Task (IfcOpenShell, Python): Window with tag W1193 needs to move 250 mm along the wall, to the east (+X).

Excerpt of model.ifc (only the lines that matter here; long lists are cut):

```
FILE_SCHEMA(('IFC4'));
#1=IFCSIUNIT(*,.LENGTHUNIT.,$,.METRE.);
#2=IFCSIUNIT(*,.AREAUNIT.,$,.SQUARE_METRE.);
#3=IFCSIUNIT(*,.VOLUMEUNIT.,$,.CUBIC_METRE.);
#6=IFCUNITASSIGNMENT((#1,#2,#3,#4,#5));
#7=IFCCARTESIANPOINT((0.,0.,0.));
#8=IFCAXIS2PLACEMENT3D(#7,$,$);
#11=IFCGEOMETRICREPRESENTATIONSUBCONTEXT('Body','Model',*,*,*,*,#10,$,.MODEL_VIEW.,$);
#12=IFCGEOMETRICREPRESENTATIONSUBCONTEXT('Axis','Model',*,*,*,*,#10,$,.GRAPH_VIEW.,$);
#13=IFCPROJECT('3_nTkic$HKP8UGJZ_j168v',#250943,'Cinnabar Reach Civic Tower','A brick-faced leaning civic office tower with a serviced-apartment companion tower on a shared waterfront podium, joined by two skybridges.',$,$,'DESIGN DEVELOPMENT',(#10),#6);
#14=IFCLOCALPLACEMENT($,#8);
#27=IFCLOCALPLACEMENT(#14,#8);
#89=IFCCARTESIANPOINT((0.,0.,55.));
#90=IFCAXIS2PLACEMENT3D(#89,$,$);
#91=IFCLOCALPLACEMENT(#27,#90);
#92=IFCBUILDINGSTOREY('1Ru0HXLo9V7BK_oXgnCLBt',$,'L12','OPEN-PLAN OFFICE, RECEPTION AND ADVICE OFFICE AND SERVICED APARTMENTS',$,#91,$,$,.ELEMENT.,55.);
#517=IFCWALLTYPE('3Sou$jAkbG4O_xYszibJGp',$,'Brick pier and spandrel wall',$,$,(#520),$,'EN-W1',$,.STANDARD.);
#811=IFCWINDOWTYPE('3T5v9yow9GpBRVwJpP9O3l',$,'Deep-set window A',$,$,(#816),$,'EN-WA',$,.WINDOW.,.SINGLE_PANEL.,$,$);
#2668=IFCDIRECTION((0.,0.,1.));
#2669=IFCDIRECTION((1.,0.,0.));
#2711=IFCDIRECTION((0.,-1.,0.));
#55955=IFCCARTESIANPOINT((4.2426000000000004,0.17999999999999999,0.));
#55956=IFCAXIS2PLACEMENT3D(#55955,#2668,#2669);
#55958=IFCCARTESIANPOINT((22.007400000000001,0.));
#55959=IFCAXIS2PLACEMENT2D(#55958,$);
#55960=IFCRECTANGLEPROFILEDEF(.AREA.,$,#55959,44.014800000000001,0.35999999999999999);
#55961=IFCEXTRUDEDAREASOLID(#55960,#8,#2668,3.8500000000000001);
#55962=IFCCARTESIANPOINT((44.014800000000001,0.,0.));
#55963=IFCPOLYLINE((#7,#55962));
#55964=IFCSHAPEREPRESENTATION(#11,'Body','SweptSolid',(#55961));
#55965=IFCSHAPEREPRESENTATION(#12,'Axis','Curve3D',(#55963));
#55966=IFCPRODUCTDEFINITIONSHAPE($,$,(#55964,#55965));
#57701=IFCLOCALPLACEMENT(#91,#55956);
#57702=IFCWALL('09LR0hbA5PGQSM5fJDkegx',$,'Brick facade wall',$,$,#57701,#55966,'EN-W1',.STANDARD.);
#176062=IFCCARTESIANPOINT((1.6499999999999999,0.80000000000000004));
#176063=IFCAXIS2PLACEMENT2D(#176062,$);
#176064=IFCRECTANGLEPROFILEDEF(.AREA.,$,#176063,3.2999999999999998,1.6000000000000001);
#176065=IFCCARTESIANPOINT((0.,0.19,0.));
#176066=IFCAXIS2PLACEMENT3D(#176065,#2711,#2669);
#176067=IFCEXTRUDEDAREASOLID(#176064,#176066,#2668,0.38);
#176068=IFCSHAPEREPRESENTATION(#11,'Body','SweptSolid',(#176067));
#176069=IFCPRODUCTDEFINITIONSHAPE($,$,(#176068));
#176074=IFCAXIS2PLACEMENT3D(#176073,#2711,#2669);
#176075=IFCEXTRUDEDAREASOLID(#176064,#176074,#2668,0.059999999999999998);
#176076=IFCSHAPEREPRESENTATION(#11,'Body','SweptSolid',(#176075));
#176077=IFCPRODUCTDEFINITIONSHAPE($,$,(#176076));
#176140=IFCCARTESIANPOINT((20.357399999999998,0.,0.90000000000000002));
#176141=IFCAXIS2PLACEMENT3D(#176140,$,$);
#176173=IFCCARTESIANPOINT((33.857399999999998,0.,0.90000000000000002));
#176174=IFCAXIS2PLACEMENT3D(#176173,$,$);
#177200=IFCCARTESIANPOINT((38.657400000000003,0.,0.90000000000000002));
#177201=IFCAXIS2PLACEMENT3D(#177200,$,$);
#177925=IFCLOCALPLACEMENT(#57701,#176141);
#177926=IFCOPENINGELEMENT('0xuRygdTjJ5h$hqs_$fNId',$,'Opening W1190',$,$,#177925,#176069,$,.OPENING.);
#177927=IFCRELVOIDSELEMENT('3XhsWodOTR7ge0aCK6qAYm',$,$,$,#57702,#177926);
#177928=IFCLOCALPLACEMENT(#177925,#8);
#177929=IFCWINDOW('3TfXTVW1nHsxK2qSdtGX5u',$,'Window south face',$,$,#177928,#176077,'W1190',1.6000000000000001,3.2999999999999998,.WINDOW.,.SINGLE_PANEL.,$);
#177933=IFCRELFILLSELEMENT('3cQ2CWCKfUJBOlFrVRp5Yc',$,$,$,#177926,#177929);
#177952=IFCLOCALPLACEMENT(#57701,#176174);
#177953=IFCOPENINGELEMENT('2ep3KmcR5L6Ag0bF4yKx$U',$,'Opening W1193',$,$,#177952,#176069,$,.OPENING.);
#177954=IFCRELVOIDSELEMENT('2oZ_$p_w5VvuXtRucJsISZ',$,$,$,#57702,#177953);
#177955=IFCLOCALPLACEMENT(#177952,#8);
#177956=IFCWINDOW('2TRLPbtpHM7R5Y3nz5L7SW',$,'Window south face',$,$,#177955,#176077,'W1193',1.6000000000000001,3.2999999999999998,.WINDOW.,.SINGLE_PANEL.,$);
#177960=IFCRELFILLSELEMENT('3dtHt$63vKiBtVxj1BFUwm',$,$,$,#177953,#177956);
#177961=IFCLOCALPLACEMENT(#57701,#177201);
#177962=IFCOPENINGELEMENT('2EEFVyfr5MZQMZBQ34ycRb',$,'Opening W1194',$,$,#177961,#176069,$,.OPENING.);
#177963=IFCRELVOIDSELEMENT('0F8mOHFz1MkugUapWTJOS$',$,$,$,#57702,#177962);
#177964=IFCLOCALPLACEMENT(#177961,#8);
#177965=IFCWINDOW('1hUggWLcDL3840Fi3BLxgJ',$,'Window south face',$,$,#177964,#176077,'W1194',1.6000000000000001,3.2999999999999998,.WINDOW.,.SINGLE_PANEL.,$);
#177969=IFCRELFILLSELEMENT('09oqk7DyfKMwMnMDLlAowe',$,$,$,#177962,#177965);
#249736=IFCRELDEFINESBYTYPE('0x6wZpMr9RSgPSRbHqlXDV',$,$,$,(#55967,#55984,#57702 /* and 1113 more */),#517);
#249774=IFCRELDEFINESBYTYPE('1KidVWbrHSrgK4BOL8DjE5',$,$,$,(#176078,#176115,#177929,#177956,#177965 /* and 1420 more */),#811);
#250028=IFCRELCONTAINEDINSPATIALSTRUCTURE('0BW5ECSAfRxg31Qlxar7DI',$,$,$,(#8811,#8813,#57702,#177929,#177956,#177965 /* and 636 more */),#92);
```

```python
import ifcopenshell
import ifcopenshell.api.geometry
import ifcopenshell.util.placement
import ifcopenshell.util.unit

model = ifcopenshell.open("model.ifc")
unit_scale = ifcopenshell.util.unit.calculate_unit_scale(model)

window = model.by_guid("2TRLPbtpHM7R5Y3nz5L7SW")
opening = window.FillsVoids[0].RelatingOpeningElement
wall = opening.VoidsElements[0].RelatingBuildingElement

wall_matrix = ifcopenshell.util.placement.get_local_placement(wall.ObjectPlacement)
shift = wall_matrix[:3, 0] * 0.25 / unit_scale
before = ifcopenshell.util.placement.get_local_placement(window.ObjectPlacement)[:3, 3].copy()

# The window is placed relative to its opening, so it follows when the opening moves.
matrix = ifcopenshell.util.placement.get_local_placement(opening.ObjectPlacement)
matrix[:3, 3] += shift
ifcopenshell.api.geometry.edit_object_placement(
    model, product=opening, matrix=matrix, is_si=False, should_transform_children=True
)

after = ifcopenshell.util.placement.get_local_placement(window.ObjectPlacement)[:3, 3]
print("window moved by", (after - before).round(3) + 0.0)

model.write("model_v2.ifc")
```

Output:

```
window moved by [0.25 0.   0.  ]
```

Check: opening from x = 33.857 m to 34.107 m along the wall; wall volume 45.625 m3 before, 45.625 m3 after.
